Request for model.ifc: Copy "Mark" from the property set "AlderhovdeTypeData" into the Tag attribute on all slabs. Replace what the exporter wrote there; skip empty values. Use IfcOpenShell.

First a look at what the model holds.

```python
import ifcopenshell
import ifcopenshell.util.element

model = ifcopenshell.open("model.ifc")
print(model.schema)
slabs = model.by_type("IfcSlab")
print(len(slabs), "slabs")
for e in slabs[:8]:
    source = ifcopenshell.util.element.get_pset(e, "AlderhovdeTypeData", "Mark")
    target = e.Tag
    print(e.id(), repr(source), repr(target), sep=" | ")
```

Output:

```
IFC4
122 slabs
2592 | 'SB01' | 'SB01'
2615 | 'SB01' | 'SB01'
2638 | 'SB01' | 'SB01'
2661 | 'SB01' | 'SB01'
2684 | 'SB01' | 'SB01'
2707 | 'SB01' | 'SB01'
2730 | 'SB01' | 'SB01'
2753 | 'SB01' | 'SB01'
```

```python
import ifcopenshell
import ifcopenshell.util.element

model = ifcopenshell.open("model.ifc")

count = 0
for e in model.by_type("IfcSlab"):
    value = ifcopenshell.util.element.get_pset(e, "AlderhovdeTypeData", "Mark")
    current = e.Tag
    if not value or not value.strip() or current == value:
        continue
    e.Tag = value
    count += 1

print(count, "slabs updated")

model.write("model_updated.ifc")
```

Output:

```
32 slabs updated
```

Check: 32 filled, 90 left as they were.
